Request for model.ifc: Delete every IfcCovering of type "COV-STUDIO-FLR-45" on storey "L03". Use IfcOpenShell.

First a look at what the model holds.

```python
import ifcopenshell
import ifcopenshell.util.element

model = ifcopenshell.open("model.ifc")
print(model.schema)
storey = next(s for s in model.by_type("IfcBuildingStorey") if s.Name == "L03")
coverings = [e for e in ifcopenshell.util.element.get_decomposition(storey) if e.is_a("IfcCovering")]
seen = {}
for e in coverings:
    element_type = ifcopenshell.util.element.get_type(e)
    name = element_type.Name if element_type not in (None, e) else None
    seen[name] = seen.get(name, 0) + 1
for name, count in sorted(seen.items(), key=str):
    print(count, "x", name)
```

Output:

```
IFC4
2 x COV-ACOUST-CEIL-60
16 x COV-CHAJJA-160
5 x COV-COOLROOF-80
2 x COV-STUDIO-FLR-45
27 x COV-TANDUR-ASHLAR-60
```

```python
import ifcopenshell
import ifcopenshell.api.root
import ifcopenshell.util.element

model = ifcopenshell.open("model.ifc")

storey = next(s for s in model.by_type("IfcBuildingStorey") if s.Name == "L03")
coverings = [e for e in ifcopenshell.util.element.get_decomposition(storey) if e.is_a("IfcCovering")]
targets = [e for e in coverings if (t := ifcopenshell.util.element.get_type(e)) not in (None, e) and t.Name == "COV-STUDIO-FLR-45"]

for e in targets:
    ifcopenshell.api.root.remove_product(model, product=e)
print(len(targets), "removed")

model.write("model_v2.ifc")
```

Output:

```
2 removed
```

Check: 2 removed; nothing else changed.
